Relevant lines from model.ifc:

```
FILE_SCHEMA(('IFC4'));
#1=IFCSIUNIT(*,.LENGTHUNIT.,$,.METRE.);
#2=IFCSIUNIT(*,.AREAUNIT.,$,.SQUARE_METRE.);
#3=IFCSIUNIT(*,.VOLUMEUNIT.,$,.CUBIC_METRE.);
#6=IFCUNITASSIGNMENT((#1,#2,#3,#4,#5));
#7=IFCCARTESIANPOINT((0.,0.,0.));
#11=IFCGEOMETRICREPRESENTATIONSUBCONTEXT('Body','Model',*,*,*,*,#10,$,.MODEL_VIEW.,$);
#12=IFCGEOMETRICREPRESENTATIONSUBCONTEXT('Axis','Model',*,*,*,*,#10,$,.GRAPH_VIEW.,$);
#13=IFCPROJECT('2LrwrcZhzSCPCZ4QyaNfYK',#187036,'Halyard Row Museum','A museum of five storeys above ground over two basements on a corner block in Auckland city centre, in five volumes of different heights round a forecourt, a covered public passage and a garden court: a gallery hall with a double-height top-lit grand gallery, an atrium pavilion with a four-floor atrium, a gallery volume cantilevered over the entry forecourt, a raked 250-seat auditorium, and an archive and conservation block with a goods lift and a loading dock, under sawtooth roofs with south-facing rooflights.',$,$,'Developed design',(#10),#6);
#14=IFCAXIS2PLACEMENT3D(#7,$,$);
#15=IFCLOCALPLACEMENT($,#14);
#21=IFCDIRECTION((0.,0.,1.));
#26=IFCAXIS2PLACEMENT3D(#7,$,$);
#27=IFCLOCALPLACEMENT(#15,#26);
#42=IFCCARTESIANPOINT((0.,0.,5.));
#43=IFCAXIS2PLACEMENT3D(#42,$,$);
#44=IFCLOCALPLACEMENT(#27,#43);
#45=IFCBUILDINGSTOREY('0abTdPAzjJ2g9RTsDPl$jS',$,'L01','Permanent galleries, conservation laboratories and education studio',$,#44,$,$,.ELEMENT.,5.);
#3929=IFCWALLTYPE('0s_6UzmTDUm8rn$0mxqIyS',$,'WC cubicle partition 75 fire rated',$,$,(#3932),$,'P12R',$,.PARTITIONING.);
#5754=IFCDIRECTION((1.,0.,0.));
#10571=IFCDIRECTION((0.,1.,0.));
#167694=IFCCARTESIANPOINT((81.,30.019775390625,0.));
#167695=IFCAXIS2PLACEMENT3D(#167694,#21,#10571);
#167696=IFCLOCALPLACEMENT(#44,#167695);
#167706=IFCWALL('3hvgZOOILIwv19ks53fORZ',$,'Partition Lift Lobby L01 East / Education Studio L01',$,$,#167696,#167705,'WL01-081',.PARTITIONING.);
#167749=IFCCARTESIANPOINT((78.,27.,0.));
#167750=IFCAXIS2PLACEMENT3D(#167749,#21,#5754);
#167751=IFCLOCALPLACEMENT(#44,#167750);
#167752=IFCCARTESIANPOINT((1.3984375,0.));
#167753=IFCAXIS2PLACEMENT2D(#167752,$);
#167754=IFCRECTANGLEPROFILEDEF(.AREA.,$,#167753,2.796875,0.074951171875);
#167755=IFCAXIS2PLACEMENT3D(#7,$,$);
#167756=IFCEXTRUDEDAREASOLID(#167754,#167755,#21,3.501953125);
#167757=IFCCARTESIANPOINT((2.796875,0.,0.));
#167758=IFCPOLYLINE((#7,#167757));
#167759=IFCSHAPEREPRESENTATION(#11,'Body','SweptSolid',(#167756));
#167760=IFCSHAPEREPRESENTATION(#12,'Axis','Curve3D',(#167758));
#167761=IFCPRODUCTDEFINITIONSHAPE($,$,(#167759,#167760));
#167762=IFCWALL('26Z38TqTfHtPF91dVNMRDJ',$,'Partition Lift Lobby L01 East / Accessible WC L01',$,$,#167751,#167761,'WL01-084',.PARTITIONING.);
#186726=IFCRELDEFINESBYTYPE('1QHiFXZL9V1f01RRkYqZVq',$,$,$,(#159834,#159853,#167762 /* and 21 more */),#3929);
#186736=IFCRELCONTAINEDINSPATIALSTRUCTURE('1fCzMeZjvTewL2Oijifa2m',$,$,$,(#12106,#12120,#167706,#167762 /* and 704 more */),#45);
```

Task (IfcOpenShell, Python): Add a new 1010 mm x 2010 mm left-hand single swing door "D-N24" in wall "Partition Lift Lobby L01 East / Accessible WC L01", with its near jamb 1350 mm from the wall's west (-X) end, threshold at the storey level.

```python
import numpy as np
import ifcopenshell
import ifcopenshell.api.feature
import ifcopenshell.api.geometry
import ifcopenshell.api.root
import ifcopenshell.api.spatial
import ifcopenshell.geom
import ifcopenshell.util.element
import ifcopenshell.util.placement
import ifcopenshell.util.representation
import ifcopenshell.util.shape
import ifcopenshell.util.unit

model = ifcopenshell.open("model.ifc")
unit_scale = ifcopenshell.util.unit.calculate_unit_scale(model)
settings = ifcopenshell.geom.settings()


def volume(element):
    """Net volume in cubic metres, openings subtracted."""
    shape = ifcopenshell.geom.create_shape(settings, element)
    return ifcopenshell.util.shape.get_volume(shape.geometry)


wall = model.by_guid("26Z38TqTfHtPF91dVNMRDJ")
storey = ifcopenshell.util.element.get_container(wall, ifc_class="IfcBuildingStorey")
context = ifcopenshell.util.representation.get_context(model, "Model", "Body", "MODEL_VIEW")
before = volume(wall)

width, height, from_end, sill = 1.01, 2.01, 1.35, 0.0  # metres

# The wall runs along its own X axis, and the end named is its -X end.
wall_shape = ifcopenshell.geom.create_shape(settings, wall)
x, y, z = ifcopenshell.util.shape.get_vertices(wall_shape.geometry).T
start = x.min() + from_end
face, thickness = float(y.min()), float(y.max() - y.min())
wall_matrix = ifcopenshell.util.placement.get_local_placement(wall.ObjectPlacement)
level = ifcopenshell.util.placement.get_local_placement(storey.ObjectPlacement)[2, 3]


def in_wall(x, y):
    """Placement at x, y metres in the wall's axes, at sill height."""
    matrix = wall_matrix.copy()
    matrix[:, 3] = wall_matrix @ np.array([x / unit_scale, y / unit_scale, 0.0, 1.0])
    matrix[2, 3] = level + sill / unit_scale
    return matrix


# Opening: a box that overshoots both wall faces by 50 mm.
opening = ifcopenshell.api.root.create_entity(model, ifc_class="IfcOpeningElement", predefined_type="OPENING")
box = ifcopenshell.api.geometry.add_wall_representation(
    model, context=context, length=width, height=height, thickness=thickness + 0.1
)
ifcopenshell.api.geometry.assign_representation(model, product=opening, representation=box)
ifcopenshell.api.geometry.edit_object_placement(model, product=opening, matrix=in_wall(start, face - 0.05), is_si=False)
ifcopenshell.api.feature.add_feature(model, feature=opening, element=wall)

door = ifcopenshell.api.root.create_entity(model, ifc_class="IfcDoor", name="D-N24", predefined_type="DOOR")
door.OverallWidth, door.OverallHeight = width / unit_scale, height / unit_scale
door.OperationType = "SINGLE_SWING_LEFT"
body = ifcopenshell.api.geometry.add_door_representation(
    model,
    context=context,
    overall_width=door.OverallWidth,
    overall_height=door.OverallHeight,
    operation_type="SINGLE_SWING_LEFT",
    lining_properties={"LiningDepth": thickness / unit_scale, "ThresholdDepth": thickness / unit_scale},
)
ifcopenshell.api.geometry.assign_representation(model, product=door, representation=body)
ifcopenshell.api.spatial.assign_container(model, products=[door], relating_structure=storey)
ifcopenshell.api.feature.add_filling(model, opening=opening, element=door)

# The lining spans the wall, so the door starts at the wall face.
ifcopenshell.api.geometry.edit_object_placement(model, product=door, matrix=in_wall(start, face), is_si=False)

after = volume(wall)

print(f"wall volume {before:.3f} -> {after:.3f} m3")

model.write("model_edited.ifc")
```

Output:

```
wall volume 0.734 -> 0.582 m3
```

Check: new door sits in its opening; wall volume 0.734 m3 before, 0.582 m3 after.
